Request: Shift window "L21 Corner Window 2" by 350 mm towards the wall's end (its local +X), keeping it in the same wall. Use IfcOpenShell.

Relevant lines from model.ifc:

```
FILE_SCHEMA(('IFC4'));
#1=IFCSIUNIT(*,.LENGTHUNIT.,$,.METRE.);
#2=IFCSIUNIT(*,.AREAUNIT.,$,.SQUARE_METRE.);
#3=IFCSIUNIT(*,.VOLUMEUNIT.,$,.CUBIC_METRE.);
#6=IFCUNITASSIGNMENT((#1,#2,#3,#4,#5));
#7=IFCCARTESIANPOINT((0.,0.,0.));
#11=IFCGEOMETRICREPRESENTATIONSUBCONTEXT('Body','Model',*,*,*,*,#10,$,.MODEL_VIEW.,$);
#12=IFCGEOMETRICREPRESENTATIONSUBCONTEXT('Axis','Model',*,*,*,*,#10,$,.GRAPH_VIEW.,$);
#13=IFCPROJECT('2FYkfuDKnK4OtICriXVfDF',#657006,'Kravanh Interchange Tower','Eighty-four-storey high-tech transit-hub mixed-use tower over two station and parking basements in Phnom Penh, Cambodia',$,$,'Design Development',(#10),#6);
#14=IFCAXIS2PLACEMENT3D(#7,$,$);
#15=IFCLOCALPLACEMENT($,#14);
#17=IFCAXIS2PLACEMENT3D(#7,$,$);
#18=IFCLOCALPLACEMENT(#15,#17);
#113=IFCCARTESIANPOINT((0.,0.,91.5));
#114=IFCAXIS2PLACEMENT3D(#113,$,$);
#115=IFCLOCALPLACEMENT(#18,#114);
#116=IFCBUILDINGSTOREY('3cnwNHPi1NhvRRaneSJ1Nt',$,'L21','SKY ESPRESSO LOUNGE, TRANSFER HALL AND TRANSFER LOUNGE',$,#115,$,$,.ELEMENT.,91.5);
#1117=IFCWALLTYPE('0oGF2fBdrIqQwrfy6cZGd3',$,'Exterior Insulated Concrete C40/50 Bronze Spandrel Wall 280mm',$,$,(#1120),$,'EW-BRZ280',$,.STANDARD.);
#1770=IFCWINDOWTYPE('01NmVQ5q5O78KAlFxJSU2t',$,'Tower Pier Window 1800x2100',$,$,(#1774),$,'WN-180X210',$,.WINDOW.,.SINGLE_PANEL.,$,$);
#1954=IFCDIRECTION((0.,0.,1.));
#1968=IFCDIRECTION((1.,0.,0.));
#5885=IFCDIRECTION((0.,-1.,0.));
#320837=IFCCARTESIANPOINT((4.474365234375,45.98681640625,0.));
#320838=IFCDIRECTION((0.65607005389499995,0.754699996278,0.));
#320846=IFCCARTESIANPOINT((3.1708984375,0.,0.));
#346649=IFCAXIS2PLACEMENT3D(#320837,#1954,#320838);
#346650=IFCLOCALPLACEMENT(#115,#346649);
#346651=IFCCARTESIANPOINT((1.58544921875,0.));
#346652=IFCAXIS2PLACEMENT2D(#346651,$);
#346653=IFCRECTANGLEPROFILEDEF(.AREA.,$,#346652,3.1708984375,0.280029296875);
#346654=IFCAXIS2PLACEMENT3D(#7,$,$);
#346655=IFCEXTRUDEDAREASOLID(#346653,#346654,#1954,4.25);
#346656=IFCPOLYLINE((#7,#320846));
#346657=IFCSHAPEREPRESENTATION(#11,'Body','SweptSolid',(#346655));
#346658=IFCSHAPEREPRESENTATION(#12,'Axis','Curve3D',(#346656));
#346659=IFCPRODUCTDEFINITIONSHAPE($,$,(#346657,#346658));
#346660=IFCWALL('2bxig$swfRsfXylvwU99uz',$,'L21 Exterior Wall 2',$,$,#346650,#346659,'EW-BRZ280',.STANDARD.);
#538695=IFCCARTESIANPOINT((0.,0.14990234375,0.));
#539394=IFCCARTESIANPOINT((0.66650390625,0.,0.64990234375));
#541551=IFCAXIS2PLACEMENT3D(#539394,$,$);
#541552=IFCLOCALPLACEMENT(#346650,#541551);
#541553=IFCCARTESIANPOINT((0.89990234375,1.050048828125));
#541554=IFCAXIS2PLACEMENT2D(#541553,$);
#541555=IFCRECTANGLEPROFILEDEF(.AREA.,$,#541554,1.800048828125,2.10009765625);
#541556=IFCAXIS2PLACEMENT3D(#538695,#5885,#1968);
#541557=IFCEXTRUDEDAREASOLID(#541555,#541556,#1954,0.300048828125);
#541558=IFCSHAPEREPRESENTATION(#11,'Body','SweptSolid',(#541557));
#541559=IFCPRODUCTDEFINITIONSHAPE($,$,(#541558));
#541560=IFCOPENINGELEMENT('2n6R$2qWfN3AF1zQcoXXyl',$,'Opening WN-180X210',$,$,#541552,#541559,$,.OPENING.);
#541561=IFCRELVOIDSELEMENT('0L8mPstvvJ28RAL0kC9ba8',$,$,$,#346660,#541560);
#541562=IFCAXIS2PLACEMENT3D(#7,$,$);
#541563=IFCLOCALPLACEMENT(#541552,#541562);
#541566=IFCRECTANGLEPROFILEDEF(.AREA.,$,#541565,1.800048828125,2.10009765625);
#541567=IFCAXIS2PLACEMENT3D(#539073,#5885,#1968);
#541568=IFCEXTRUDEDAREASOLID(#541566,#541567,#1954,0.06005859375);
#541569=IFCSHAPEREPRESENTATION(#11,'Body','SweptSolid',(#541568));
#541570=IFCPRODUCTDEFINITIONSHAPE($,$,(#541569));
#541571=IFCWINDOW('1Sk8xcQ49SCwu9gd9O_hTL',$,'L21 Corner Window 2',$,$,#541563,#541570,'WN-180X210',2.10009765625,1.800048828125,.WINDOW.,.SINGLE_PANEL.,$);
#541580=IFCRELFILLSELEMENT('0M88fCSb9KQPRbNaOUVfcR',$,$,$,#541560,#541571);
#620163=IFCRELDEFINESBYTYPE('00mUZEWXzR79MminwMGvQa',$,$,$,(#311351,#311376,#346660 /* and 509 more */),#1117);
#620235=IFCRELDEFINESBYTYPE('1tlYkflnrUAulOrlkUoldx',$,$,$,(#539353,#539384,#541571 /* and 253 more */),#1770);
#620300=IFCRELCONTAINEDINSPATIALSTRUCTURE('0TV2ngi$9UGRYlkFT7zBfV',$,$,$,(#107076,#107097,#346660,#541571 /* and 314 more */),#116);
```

```python
import ifcopenshell
import ifcopenshell.api.geometry
import ifcopenshell.util.placement
import ifcopenshell.util.unit

model = ifcopenshell.open("model.ifc")
unit_scale = ifcopenshell.util.unit.calculate_unit_scale(model)

window = model.by_id(541571)
opening = window.FillsVoids[0].RelatingOpeningElement
wall = opening.VoidsElements[0].RelatingBuildingElement

wall_matrix = ifcopenshell.util.placement.get_local_placement(wall.ObjectPlacement)
shift = wall_matrix[:3, 0] * 0.35 / unit_scale
before = ifcopenshell.util.placement.get_local_placement(window.ObjectPlacement)[:3, 3].copy()

# The window is placed relative to its opening, so it follows when the opening moves.
matrix = ifcopenshell.util.placement.get_local_placement(opening.ObjectPlacement)
matrix[:3, 3] += shift
ifcopenshell.api.geometry.edit_object_placement(
    model, product=opening, matrix=matrix, is_si=False, should_transform_children=True
)

after = ifcopenshell.util.placement.get_local_placement(window.ObjectPlacement)[:3, 3]
print("window moved by", (after - before).round(3) + 0.0)

model.write("model-out.ifc")
```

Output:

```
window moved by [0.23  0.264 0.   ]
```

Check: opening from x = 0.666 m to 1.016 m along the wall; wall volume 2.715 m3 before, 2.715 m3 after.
